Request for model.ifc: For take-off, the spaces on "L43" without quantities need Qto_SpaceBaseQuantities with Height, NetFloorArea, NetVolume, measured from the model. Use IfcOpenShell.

First a look at what the model holds.

```python
import ifcopenshell
import ifcopenshell.util.element
import ifcopenshell.util.unit

model = ifcopenshell.open("model.ifc")
print(model.schema)
for unit_type in ("LENGTHUNIT", "AREAUNIT", "VOLUMEUNIT"):
    print(unit_type, ifcopenshell.util.unit.calculate_unit_scale(model, unit_type))
storey = next(s for s in model.by_type("IfcBuildingStorey") if s.Name == "L43")
spaces = [e for e in ifcopenshell.util.element.get_decomposition(storey) if e.is_a("IfcSpace")]
for e in sorted(spaces, key=lambda e: e.id()):
    print(e.id(), e.is_a(), e.Name, list(ifcopenshell.util.element.get_psets(e, qtos_only=True)), sep=" | ")
```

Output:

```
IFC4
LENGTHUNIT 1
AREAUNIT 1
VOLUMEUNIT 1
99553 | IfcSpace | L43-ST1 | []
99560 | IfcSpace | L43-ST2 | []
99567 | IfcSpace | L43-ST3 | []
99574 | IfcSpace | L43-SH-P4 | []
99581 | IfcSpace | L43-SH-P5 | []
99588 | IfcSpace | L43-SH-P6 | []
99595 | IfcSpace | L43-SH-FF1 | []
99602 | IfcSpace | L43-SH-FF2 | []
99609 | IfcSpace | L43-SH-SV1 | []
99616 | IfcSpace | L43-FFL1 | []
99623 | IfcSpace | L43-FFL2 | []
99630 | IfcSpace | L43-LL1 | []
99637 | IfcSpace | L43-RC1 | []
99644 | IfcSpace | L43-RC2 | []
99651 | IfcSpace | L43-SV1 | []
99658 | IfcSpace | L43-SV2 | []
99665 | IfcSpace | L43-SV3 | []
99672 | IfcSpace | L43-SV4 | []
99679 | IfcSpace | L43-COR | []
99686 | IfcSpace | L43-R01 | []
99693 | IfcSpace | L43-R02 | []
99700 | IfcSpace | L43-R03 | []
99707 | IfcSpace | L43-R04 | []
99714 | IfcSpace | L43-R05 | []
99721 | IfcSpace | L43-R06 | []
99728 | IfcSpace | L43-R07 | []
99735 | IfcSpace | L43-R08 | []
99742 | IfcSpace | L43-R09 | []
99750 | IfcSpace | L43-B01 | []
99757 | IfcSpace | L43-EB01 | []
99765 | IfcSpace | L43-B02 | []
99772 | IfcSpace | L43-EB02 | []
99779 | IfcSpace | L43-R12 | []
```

```python
import ifcopenshell
import ifcopenshell.api.pset
import ifcopenshell.geom
import ifcopenshell.util.element
import ifcopenshell.util.shape
import ifcopenshell.util.unit

model = ifcopenshell.open("model.ifc")
unit_scale = ifcopenshell.util.unit.calculate_unit_scale(model)
area_scale = ifcopenshell.util.unit.calculate_unit_scale(model, "AREAUNIT")
volume_scale = ifcopenshell.util.unit.calculate_unit_scale(model, "VOLUMEUNIT")
settings = ifcopenshell.geom.settings()

storey = next(s for s in model.by_type("IfcBuildingStorey") if s.Name == "L43")
spaces = [e for e in ifcopenshell.util.element.get_decomposition(storey) if e.is_a("IfcSpace")]

for e in sorted(spaces, key=lambda e: e.id()):
    if ifcopenshell.util.element.get_psets(e, qtos_only=True, should_inherit=False):
        continue
    # Geometry comes back in metres, in the element's own axes.
    shape = ifcopenshell.geom.create_shape(settings, e)
    values = {
        "Height": ifcopenshell.util.shape.get_z(shape.geometry) / unit_scale,
        "NetFloorArea": ifcopenshell.util.shape.get_footprint_area(shape.geometry) / area_scale,
        "NetVolume": ifcopenshell.util.shape.get_volume(shape.geometry) / volume_scale,
    }
    qto = ifcopenshell.api.pset.add_qto(model, product=e, name="Qto_SpaceBaseQuantities")
    ifcopenshell.api.pset.edit_qto(model, qto=qto, properties=values)
    print(e.id(), {k: round(v, 3) for k, v in values.items()})

model.write("model_rev.ifc")
```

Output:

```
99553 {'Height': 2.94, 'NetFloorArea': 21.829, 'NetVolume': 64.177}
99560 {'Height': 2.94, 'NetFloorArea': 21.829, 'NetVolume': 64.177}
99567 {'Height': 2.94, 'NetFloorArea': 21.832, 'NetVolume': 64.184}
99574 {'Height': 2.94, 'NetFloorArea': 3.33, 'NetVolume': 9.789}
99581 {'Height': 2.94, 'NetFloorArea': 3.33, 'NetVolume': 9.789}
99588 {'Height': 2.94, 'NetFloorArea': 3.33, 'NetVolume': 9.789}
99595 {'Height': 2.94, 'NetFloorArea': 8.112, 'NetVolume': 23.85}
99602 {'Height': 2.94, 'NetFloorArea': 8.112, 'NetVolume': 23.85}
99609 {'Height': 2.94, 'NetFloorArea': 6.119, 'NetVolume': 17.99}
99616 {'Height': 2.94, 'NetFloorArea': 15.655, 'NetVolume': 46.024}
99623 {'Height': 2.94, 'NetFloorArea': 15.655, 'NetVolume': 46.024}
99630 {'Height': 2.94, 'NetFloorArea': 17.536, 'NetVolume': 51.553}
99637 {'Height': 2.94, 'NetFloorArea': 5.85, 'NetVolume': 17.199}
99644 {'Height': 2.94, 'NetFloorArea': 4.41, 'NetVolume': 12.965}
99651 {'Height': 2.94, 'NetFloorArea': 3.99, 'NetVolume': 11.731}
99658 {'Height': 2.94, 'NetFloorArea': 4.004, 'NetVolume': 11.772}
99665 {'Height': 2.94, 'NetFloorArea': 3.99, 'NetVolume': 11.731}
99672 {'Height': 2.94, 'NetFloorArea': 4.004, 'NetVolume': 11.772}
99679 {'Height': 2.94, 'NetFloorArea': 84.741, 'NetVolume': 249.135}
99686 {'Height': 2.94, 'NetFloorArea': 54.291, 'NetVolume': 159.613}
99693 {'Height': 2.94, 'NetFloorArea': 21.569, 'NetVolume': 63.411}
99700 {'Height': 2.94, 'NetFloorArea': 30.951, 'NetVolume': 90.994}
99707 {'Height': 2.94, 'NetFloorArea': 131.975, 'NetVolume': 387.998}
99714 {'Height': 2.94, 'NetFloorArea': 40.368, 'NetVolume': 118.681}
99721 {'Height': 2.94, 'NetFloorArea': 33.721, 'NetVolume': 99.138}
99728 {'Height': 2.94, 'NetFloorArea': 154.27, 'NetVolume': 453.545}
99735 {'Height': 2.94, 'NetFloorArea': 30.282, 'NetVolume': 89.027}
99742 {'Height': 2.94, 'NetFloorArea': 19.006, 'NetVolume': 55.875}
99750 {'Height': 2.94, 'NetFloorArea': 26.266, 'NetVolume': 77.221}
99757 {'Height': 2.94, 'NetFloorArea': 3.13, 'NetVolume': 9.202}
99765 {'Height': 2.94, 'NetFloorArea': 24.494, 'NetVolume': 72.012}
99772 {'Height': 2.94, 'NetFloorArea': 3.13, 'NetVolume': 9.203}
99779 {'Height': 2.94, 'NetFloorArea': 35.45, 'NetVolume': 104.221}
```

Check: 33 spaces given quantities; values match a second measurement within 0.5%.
